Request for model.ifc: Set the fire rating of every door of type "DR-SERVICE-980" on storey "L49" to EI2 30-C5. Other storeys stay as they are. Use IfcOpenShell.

First a look at what the model holds.

```python
import ifcopenshell
import ifcopenshell.util.element

model = ifcopenshell.open("model.ifc")
print(model.schema)
storey = next(s for s in model.by_type("IfcBuildingStorey") if s.Name == "L49")
doors = [e for e in ifcopenshell.util.element.get_decomposition(storey) if e.is_a("IfcDoor")]
seen = {}
for e in doors:
    element_type = ifcopenshell.util.element.get_type(e)
    key = (element_type.Name if element_type != e and element_type else None, ifcopenshell.util.element.get_pset(e, "Pset_DoorCommon", "FireRating"))
    seen[key] = seen.get(key, 0) + 1
for (name, value), count in sorted(seen.items(), key=str):
    print(count, "x", name, "|", value)
```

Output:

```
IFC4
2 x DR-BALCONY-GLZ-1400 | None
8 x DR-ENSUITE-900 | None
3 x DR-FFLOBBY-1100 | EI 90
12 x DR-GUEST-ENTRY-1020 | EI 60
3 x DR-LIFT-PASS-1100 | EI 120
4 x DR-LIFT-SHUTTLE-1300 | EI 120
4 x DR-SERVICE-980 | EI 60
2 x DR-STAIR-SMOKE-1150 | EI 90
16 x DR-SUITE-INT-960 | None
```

```python
import ifcopenshell
import ifcopenshell.api.pset
import ifcopenshell.util.element

model = ifcopenshell.open("model.ifc")

storey = next(s for s in model.by_type("IfcBuildingStorey") if s.Name == "L49")
doors = [e for e in ifcopenshell.util.element.get_decomposition(storey) if e.is_a("IfcDoor")]

count = 0
for e in doors:
    element_type = ifcopenshell.util.element.get_type(e)
    if element_type in (None, e) or element_type.Name != "DR-SERVICE-980":
        continue
    # add_pset returns the element's existing set when there is one.
    pset = ifcopenshell.api.pset.add_pset(model, product=e, name="Pset_DoorCommon")
    ifcopenshell.api.pset.edit_pset(model, pset=pset, properties={"FireRating": "EI2 30-C5"})
    count += 1

print(count, "doors updated")

model.write("model_updated.ifc")
```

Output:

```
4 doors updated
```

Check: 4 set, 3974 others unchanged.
